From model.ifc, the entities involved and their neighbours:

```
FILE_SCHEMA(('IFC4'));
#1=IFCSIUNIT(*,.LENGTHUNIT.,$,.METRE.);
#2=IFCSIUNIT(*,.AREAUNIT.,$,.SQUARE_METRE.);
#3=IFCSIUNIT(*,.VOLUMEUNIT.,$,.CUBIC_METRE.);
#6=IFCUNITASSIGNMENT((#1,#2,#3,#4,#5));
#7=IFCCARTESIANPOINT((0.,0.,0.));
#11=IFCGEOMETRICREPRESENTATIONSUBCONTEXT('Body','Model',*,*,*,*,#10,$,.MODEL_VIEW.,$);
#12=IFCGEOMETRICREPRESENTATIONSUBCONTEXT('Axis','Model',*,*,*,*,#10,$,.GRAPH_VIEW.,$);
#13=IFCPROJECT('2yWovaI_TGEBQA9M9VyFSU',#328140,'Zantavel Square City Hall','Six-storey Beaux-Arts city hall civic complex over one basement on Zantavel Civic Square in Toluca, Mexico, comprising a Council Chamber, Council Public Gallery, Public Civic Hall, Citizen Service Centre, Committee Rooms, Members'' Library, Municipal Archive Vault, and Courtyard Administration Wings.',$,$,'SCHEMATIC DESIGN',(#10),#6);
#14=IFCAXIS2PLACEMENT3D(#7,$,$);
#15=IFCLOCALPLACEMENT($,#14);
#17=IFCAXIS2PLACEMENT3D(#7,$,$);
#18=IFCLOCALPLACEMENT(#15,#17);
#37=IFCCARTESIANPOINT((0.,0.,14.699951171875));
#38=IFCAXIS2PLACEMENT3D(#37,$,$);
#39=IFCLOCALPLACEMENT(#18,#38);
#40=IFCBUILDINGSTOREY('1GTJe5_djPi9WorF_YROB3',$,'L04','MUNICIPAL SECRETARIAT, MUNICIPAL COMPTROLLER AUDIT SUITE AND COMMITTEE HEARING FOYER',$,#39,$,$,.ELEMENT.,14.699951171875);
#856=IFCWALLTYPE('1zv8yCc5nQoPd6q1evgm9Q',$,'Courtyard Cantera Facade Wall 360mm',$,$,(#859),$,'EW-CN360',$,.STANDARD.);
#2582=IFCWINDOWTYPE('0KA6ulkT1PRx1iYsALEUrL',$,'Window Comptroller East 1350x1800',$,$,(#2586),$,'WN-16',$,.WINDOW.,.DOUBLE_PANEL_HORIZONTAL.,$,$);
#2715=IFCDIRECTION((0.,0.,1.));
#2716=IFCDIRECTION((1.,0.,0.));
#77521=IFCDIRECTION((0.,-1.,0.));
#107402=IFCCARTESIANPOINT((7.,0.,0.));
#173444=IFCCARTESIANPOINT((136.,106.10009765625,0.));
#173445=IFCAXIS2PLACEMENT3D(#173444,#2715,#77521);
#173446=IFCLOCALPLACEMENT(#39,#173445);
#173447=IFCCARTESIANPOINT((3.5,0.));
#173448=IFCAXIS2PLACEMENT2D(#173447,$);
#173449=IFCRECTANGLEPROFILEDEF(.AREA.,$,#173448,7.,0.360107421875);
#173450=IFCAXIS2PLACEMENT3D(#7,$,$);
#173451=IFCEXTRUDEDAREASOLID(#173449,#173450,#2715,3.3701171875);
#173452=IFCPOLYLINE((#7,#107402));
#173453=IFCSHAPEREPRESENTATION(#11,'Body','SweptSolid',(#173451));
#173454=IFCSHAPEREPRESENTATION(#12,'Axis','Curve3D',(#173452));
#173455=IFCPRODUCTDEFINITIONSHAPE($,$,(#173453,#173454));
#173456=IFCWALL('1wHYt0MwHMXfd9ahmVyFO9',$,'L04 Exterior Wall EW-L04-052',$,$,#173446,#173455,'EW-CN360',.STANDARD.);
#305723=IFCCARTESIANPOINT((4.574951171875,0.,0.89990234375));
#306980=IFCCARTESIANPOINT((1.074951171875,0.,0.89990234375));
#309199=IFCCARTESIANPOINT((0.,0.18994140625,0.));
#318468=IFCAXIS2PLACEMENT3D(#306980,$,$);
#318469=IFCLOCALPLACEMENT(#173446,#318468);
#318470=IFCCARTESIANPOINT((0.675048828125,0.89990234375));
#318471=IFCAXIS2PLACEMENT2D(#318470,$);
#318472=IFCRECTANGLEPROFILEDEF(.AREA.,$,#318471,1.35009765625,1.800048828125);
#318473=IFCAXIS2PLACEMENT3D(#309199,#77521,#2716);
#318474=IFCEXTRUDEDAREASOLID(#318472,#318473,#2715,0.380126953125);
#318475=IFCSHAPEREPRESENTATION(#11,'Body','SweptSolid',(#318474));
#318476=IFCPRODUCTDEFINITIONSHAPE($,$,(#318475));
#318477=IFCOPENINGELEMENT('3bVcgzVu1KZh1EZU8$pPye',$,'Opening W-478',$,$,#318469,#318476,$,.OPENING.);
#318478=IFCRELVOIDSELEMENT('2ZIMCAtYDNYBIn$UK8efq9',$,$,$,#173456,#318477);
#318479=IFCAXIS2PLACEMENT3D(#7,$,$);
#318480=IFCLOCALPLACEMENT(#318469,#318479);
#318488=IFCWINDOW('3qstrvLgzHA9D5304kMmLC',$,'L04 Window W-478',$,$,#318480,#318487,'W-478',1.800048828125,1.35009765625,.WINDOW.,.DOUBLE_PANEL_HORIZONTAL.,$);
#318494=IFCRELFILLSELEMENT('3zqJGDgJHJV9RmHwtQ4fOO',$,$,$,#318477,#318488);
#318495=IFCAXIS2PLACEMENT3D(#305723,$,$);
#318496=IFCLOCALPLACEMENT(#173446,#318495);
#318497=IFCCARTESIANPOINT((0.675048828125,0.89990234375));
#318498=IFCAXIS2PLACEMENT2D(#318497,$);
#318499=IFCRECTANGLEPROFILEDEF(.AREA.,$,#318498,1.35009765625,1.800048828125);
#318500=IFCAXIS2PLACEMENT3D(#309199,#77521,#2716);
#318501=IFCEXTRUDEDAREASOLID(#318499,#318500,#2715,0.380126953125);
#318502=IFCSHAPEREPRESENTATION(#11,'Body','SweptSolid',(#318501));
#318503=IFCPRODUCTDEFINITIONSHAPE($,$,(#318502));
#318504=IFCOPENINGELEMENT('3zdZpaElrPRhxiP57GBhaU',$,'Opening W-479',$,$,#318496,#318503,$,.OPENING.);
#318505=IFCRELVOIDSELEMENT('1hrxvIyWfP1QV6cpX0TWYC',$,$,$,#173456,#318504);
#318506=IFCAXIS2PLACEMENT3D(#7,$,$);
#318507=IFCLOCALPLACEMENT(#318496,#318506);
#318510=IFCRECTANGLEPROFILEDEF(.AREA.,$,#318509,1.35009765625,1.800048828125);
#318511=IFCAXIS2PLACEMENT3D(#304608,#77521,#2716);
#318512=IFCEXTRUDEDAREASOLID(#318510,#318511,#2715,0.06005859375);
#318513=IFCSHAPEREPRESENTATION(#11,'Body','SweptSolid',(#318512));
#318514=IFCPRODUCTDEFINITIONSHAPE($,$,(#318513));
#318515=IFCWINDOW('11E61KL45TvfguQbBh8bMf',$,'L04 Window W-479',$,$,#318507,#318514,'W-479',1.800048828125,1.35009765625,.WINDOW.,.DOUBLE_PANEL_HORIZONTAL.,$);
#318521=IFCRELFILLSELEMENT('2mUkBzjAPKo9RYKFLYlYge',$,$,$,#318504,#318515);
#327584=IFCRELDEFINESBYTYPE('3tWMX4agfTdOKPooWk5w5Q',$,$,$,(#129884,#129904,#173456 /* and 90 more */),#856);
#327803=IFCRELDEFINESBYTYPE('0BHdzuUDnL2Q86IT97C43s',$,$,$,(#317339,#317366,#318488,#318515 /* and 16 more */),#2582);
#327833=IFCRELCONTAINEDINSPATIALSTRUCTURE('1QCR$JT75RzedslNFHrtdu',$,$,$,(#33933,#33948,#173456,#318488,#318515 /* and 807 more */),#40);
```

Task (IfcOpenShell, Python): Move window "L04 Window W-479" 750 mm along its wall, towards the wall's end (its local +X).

```python
import ifcopenshell
import ifcopenshell.api.geometry
import ifcopenshell.util.placement
import ifcopenshell.util.unit

model = ifcopenshell.open("model.ifc")
unit_scale = ifcopenshell.util.unit.calculate_unit_scale(model)

window = model.by_guid("11E61KL45TvfguQbBh8bMf")
opening = window.FillsVoids[0].RelatingOpeningElement
wall = opening.VoidsElements[0].RelatingBuildingElement

wall_matrix = ifcopenshell.util.placement.get_local_placement(wall.ObjectPlacement)
shift = wall_matrix[:3, 0] * 0.75 / unit_scale
before = ifcopenshell.util.placement.get_local_placement(window.ObjectPlacement)[:3, 3].copy()

# The window is placed relative to its opening, so it follows when the opening moves.
matrix = ifcopenshell.util.placement.get_local_placement(opening.ObjectPlacement)
matrix[:3, 3] += shift
ifcopenshell.api.geometry.edit_object_placement(
    model, product=opening, matrix=matrix, is_si=False, should_transform_children=True
)

after = ifcopenshell.util.placement.get_local_placement(window.ObjectPlacement)[:3, 3]
print("window moved by", (after - before).round(3) + 0.0)

model.write("model_updated.ifc")
```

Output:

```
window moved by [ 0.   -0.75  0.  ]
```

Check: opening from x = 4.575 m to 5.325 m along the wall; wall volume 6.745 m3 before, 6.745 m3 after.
